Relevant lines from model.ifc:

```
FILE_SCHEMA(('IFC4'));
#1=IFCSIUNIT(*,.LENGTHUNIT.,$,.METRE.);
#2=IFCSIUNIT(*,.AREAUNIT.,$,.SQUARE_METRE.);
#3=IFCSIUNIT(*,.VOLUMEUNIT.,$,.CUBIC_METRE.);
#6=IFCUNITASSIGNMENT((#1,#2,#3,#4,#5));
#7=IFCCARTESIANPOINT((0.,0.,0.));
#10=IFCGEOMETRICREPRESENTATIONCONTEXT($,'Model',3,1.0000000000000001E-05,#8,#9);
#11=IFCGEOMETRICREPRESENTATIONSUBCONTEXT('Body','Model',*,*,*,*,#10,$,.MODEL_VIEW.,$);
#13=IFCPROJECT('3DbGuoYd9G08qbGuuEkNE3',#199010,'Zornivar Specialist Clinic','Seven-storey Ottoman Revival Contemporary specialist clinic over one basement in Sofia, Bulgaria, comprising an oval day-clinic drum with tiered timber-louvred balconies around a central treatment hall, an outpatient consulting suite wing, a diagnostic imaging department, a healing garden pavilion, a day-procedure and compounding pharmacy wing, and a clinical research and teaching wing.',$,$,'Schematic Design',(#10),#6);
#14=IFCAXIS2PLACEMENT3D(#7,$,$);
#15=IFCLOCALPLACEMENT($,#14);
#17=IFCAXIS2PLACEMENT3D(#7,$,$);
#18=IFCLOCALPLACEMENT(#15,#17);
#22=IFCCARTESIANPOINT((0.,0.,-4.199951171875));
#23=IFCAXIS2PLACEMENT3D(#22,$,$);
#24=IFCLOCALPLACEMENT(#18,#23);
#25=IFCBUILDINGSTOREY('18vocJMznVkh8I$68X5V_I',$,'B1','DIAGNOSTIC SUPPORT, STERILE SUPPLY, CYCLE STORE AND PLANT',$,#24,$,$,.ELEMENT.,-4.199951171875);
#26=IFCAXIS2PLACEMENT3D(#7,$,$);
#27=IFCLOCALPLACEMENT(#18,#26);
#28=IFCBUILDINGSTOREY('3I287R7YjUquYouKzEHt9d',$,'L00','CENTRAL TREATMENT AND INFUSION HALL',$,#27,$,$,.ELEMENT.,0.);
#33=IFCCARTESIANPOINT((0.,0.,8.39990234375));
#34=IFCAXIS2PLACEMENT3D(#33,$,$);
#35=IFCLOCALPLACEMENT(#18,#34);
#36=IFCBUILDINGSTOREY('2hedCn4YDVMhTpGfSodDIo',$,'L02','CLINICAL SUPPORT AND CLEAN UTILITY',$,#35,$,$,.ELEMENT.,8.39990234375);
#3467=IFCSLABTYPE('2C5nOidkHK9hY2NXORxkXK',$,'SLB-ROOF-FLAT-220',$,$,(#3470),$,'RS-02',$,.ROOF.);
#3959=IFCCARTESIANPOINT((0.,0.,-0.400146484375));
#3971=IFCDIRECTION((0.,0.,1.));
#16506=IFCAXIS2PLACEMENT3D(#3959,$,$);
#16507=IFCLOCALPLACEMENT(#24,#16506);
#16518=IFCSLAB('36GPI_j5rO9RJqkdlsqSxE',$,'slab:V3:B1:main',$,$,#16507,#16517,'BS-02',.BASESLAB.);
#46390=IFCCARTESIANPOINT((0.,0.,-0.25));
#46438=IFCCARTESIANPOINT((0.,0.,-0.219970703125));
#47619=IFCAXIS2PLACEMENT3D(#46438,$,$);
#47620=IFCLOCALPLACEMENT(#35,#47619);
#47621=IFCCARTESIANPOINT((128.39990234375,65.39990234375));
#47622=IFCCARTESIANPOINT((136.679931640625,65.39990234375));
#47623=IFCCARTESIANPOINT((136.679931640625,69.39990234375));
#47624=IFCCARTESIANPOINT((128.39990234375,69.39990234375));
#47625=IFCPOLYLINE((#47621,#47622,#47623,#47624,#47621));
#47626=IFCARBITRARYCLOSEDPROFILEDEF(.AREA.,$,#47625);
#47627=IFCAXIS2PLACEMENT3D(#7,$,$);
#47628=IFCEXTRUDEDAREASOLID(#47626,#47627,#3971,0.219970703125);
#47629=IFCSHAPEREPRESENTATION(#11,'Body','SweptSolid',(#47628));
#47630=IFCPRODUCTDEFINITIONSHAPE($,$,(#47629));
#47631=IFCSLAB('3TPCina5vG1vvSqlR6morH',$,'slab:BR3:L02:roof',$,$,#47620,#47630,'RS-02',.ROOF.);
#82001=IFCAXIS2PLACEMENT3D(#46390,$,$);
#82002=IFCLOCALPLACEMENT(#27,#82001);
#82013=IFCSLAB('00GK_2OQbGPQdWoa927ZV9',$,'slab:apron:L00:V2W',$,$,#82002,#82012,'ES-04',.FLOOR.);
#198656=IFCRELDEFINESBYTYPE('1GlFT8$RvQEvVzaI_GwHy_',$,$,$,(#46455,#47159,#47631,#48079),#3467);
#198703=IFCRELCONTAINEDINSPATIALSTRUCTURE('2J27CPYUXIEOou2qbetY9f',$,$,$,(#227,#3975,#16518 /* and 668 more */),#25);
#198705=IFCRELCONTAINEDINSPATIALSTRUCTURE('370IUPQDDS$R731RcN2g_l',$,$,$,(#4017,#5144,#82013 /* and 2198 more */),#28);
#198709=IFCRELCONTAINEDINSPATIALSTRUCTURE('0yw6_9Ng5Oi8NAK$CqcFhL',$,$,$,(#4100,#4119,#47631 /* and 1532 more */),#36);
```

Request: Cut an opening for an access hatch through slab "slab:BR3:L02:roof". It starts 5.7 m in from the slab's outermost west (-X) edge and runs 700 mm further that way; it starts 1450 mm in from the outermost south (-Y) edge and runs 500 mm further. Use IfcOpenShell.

```python
import numpy as np
import ifcopenshell
import ifcopenshell.api.feature
import ifcopenshell.api.geometry
import ifcopenshell.api.root
import ifcopenshell.geom
import ifcopenshell.util.placement
import ifcopenshell.util.representation
import ifcopenshell.util.shape
import ifcopenshell.util.unit

model = ifcopenshell.open("model.ifc")
unit_scale = ifcopenshell.util.unit.calculate_unit_scale(model)
settings = ifcopenshell.geom.settings()


def volume(element):
    """Net volume in cubic metres, openings subtracted."""
    shape = ifcopenshell.geom.create_shape(settings, element)
    return ifcopenshell.util.shape.get_volume(shape.geometry)


slab = model.by_guid("3TPCina5vG1vvSqlR6morH")
before = volume(slab)

# Extent in the slab's own axes, in metres. The edges named are its -X and -Y sides.
slab_shape = ifcopenshell.geom.create_shape(settings, slab)
vertices = ifcopenshell.util.shape.get_vertices(slab_shape.geometry)
x_min, y_min, bottom = vertices.min(axis=0)
top = vertices[:, 2].max()

opening = ifcopenshell.api.root.create_entity(model, ifc_class="IfcOpeningElement", name="Access hatch opening", predefined_type="OPENING")
context = ifcopenshell.util.representation.get_context(model, "Model", "Body", "MODEL_VIEW")
width, depth = 0.7, 0.5
outline = [(0.0, 0.0), (width, 0.0), (width, depth), (0.0, depth), (0.0, 0.0)]
# Overshoot both faces by 50 mm so the cut is clean.
shape = ifcopenshell.api.geometry.add_slab_representation(
    model, context=context, depth=top - bottom + 0.1, polyline=outline
)
ifcopenshell.api.geometry.assign_representation(model, product=opening, representation=shape)

matrix = ifcopenshell.util.placement.get_local_placement(slab.ObjectPlacement)
matrix[:, 3] = matrix @ np.append(np.array([x_min + 5.7, y_min + 1.45, bottom - 0.05]) / unit_scale, 1.0)
ifcopenshell.api.geometry.edit_object_placement(model, product=opening, matrix=matrix, is_si=False)
ifcopenshell.api.feature.add_feature(model, feature=opening, element=slab)

after = volume(slab)

print(f"slab volume {before:.3f} -> {after:.3f} m3")

model.write("model_rev.ifc")
```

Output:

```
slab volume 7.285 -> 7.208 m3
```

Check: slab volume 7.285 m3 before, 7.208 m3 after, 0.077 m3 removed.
